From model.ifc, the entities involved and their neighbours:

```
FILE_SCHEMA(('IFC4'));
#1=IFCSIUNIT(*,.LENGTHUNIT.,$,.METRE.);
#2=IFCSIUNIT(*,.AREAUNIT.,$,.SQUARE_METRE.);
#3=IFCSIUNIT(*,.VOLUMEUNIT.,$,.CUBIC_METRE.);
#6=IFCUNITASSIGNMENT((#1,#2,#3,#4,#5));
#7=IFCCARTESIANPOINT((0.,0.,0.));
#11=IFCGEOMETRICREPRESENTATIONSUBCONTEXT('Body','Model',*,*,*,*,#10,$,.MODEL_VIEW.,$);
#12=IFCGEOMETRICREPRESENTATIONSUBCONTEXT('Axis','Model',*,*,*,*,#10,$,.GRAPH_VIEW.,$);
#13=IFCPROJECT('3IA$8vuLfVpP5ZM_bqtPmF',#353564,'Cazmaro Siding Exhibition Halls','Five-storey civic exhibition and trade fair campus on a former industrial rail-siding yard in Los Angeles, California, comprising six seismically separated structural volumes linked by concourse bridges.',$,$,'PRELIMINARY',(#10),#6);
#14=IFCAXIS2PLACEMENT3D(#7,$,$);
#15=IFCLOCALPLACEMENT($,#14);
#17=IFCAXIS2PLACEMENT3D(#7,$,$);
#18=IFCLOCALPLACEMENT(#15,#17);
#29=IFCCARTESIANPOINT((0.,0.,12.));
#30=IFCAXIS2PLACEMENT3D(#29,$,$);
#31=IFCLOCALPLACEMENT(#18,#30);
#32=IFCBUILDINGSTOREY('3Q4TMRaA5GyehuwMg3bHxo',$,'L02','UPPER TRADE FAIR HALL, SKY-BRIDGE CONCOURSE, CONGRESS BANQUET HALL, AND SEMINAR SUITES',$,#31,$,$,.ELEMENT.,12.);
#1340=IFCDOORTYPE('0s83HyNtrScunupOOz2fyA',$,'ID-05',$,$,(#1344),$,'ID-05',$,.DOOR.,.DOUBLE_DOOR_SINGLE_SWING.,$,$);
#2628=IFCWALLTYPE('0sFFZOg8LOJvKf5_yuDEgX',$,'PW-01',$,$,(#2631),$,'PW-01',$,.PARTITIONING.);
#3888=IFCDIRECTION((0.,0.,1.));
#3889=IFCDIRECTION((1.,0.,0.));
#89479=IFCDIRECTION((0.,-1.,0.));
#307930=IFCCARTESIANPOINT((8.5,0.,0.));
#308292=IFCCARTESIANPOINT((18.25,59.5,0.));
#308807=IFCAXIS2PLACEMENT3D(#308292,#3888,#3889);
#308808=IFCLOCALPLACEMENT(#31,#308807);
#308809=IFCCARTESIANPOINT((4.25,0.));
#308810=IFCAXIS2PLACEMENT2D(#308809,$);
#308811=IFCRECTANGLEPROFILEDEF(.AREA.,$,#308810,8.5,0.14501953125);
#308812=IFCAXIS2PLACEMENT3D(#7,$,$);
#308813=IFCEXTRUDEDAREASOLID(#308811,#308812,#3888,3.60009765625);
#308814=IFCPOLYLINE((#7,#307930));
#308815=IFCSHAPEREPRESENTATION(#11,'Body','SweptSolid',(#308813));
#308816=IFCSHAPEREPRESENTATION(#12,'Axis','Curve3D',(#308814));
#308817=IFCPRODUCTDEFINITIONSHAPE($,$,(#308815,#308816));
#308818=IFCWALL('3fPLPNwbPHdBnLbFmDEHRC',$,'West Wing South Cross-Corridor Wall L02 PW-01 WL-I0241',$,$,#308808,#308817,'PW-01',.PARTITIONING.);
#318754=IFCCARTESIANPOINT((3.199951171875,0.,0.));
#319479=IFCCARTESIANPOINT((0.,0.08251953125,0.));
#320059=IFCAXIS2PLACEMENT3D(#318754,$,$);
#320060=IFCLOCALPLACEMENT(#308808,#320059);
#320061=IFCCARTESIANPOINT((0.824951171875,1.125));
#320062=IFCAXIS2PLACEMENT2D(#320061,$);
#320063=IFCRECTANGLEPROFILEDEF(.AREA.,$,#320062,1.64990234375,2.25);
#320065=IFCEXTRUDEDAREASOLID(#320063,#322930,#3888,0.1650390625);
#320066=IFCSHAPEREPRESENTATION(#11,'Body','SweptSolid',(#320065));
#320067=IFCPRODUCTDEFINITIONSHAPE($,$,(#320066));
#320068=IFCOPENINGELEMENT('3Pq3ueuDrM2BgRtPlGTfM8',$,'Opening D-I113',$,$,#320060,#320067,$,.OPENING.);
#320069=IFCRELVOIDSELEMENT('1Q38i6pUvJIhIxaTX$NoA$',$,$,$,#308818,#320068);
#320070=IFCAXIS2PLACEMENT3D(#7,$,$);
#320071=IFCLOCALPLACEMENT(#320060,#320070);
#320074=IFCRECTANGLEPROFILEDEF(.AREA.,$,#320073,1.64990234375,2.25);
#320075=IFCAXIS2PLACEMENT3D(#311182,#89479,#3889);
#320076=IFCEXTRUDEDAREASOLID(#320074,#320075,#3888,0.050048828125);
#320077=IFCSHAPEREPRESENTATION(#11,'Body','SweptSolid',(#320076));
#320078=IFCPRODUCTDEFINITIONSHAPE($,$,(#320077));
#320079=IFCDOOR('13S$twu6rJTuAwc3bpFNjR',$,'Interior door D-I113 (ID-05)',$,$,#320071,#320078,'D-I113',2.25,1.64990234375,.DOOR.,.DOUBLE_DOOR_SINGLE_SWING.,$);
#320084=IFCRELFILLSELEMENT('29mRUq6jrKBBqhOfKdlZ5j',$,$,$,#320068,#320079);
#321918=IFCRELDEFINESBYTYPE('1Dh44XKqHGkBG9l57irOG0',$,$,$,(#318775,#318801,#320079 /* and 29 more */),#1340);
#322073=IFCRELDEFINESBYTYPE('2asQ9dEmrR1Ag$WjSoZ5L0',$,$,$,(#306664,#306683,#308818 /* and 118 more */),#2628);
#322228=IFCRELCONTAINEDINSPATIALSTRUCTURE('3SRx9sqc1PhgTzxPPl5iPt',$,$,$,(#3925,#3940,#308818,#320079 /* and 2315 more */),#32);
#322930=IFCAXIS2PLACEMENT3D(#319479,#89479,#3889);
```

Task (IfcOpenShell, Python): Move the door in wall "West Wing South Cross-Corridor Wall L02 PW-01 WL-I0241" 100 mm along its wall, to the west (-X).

```python
import ifcopenshell
import ifcopenshell.api.geometry
import ifcopenshell.util.placement

model = ifcopenshell.open("model.ifc")

door = model.by_id(320079)
opening = door.FillsVoids[0].RelatingOpeningElement
wall = opening.VoidsElements[0].RelatingBuildingElement

wall_matrix = ifcopenshell.util.placement.get_local_placement(wall.ObjectPlacement)
shift = wall_matrix[:3, 0] * -0.1
before = ifcopenshell.util.placement.get_local_placement(door.ObjectPlacement)[:3, 3].copy()

# The door is placed relative to its opening, so it follows when the opening moves.
matrix = ifcopenshell.util.placement.get_local_placement(opening.ObjectPlacement)
matrix[:3, 3] += shift
ifcopenshell.api.geometry.edit_object_placement(
    model, product=opening, matrix=matrix, is_si=False, should_transform_children=True
)

after = ifcopenshell.util.placement.get_local_placement(door.ObjectPlacement)[:3, 3]
print("door moved by", (after - before).round(3) + 0.0)

model.write("model_edited.ifc")
```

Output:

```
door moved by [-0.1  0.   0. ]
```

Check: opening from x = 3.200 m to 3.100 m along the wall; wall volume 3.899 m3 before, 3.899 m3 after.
